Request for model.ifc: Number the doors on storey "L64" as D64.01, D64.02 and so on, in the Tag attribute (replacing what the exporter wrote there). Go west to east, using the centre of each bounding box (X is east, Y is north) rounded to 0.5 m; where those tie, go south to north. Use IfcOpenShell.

First a look at what the model holds.

```python
import ifcopenshell
import ifcopenshell.util.element
import ifcopenshell.util.placement

model = ifcopenshell.open("model.ifc")
print(model.schema)
storey = next(s for s in model.by_type("IfcBuildingStorey") if s.Name == "L64")
doors = [e for e in ifcopenshell.util.element.get_decomposition(storey) if e.is_a("IfcDoor")]
for e in sorted(doors, key=lambda e: e.id()):
    origin = ifcopenshell.util.placement.get_local_placement(e.ObjectPlacement)[:3, 3]
    print(e.id(), e.Tag, e.Name, origin.round(2) + 0.0, sep=" | ")
```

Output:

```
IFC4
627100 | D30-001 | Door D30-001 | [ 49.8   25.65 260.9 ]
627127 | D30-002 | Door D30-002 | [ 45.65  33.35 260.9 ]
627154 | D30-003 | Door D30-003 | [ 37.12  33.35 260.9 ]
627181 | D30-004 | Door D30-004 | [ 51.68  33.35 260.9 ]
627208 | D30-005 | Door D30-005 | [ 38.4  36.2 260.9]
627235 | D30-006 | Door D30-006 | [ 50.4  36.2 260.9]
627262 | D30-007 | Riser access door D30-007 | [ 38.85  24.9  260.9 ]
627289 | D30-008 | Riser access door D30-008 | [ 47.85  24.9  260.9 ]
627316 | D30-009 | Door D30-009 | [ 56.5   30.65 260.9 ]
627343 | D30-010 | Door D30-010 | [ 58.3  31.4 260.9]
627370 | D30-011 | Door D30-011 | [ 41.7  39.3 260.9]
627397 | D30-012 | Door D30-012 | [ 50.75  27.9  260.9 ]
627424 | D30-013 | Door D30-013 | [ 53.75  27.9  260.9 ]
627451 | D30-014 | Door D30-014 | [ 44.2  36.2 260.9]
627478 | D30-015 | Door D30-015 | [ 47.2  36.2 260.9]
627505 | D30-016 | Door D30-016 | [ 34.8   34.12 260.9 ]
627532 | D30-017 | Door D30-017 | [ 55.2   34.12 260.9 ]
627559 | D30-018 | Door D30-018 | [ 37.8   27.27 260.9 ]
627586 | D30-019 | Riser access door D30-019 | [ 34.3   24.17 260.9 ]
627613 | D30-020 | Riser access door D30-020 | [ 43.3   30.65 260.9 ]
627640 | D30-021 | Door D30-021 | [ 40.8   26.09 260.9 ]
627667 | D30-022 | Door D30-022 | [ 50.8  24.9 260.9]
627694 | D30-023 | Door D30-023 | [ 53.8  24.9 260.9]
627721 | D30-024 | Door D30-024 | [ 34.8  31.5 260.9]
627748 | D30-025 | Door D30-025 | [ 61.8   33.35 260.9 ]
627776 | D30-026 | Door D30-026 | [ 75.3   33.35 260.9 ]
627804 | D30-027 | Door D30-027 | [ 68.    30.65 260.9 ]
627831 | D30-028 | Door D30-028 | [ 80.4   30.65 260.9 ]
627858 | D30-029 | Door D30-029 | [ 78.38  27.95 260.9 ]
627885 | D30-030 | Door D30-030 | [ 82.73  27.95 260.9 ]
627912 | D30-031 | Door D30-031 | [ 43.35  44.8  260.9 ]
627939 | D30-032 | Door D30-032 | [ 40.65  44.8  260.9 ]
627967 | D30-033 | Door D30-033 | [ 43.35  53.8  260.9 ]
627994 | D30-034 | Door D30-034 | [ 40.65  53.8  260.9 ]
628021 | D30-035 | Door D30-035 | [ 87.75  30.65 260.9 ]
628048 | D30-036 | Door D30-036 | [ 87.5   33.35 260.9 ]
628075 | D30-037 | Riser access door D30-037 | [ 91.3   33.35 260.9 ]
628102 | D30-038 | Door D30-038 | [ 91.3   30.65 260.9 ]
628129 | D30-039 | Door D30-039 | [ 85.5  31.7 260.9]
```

```python
import ifcopenshell
import ifcopenshell.geom
import ifcopenshell.util.element
import ifcopenshell.util.shape

model = ifcopenshell.open("model.ifc")
settings = ifcopenshell.geom.settings()
settings.set("use-world-coords", True)


def centre(element):
    shape = ifcopenshell.geom.create_shape(settings, element)
    return ifcopenshell.util.shape.get_bbox_centroid(shape.geometry)


storey = next(s for s in model.by_type("IfcBuildingStorey") if s.Name == "L64")
doors = [e for e in ifcopenshell.util.element.get_decomposition(storey) if e.is_a("IfcDoor")]

# Insertion points can sit at a corner or the storey origin, so sort by the geometry (in metres).
centres = {e: centre(e) for e in doors}
doors.sort(key=lambda e: (round(centres[e][0] / 0.5), centres[e][1]))

for i, e in enumerate(doors, start=1):
    number = f"D64.{i:02d}"
    e.Tag = number
    print(e.id(), number)

model.write("model_updated.ifc")
```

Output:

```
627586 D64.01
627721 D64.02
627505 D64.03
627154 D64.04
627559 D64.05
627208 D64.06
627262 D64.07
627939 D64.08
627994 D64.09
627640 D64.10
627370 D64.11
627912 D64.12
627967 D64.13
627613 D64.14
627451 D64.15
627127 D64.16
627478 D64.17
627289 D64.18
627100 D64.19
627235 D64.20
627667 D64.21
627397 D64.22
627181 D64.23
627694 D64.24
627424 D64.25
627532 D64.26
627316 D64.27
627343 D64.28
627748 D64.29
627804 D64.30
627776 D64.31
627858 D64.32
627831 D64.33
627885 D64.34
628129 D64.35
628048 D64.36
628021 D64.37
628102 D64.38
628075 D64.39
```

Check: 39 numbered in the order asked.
